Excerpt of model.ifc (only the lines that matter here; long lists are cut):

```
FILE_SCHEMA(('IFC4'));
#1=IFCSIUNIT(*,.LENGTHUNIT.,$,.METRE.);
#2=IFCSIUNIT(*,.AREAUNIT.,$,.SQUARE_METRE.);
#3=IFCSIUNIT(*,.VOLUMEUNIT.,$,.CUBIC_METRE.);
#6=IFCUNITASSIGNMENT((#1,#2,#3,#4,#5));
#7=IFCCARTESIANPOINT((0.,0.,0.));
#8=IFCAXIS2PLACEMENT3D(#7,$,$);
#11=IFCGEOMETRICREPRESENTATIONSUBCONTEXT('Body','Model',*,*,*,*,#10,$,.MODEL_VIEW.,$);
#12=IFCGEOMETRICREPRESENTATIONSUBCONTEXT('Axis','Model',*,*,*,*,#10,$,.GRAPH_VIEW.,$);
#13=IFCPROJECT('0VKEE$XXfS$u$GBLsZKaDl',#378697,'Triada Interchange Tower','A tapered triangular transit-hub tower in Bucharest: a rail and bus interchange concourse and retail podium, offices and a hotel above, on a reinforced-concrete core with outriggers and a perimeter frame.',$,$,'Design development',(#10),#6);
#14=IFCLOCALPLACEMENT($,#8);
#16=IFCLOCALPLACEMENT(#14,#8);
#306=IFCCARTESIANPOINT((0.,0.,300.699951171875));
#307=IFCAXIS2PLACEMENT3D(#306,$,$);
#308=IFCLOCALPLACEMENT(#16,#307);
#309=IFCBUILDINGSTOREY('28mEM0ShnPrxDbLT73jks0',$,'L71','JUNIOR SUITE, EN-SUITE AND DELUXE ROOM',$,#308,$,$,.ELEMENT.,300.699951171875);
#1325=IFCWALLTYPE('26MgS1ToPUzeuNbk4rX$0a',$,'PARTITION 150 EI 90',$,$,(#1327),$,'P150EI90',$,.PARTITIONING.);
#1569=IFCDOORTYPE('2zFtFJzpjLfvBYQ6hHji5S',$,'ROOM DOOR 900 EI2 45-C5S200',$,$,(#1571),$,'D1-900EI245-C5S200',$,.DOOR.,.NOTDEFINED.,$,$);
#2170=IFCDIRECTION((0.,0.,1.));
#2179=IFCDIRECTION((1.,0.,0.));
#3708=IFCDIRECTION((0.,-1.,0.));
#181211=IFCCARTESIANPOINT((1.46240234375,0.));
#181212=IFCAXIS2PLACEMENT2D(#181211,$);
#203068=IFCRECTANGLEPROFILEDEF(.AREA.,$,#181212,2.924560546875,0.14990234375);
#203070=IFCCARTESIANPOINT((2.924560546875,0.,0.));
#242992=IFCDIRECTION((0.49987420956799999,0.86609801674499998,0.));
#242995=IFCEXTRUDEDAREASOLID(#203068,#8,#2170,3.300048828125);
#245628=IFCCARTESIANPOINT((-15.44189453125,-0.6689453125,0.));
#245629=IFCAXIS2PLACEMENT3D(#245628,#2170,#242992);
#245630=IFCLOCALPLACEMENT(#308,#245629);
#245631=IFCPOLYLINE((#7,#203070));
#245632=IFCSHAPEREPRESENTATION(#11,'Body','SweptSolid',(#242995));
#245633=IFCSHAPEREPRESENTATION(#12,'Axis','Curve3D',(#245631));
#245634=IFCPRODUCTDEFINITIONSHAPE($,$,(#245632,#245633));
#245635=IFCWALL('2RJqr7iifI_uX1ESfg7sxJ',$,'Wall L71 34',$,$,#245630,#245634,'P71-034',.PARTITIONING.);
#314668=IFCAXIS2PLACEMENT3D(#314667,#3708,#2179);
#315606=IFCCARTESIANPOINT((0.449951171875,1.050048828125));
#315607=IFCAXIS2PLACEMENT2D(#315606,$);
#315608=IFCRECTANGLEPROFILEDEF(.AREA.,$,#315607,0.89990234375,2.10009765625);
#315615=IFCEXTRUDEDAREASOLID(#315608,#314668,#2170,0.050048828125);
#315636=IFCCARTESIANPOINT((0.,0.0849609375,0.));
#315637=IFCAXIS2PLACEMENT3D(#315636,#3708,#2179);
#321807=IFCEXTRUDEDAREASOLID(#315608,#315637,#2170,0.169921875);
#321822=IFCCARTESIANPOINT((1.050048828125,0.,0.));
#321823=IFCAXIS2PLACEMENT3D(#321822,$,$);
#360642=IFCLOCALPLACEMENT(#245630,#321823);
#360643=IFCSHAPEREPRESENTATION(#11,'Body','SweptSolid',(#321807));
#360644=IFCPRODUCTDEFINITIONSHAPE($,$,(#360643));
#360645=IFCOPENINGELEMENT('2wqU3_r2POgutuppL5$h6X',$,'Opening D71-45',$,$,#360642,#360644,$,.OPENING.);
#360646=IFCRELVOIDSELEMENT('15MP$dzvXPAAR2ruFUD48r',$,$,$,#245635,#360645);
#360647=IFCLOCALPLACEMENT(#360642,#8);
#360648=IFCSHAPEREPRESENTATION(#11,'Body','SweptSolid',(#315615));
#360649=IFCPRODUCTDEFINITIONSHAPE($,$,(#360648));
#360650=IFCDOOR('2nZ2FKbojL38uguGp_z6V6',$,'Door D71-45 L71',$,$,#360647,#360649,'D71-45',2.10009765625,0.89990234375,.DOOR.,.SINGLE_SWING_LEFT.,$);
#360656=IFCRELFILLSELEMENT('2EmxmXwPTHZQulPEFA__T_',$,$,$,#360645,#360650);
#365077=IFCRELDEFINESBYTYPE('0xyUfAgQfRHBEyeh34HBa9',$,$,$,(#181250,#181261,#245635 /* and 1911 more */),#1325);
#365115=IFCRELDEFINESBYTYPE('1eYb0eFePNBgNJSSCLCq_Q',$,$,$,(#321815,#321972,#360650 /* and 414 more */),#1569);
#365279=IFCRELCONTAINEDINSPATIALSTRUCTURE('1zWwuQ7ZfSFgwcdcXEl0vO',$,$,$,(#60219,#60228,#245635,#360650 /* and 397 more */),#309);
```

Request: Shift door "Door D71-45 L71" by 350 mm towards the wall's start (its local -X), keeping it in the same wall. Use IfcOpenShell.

```python
import ifcopenshell
import ifcopenshell.api.geometry
import ifcopenshell.util.placement
import ifcopenshell.util.unit

model = ifcopenshell.open("model.ifc")
unit_scale = ifcopenshell.util.unit.calculate_unit_scale(model)

door = model.by_guid("2nZ2FKbojL38uguGp_z6V6")
opening = door.FillsVoids[0].RelatingOpeningElement
wall = opening.VoidsElements[0].RelatingBuildingElement

wall_matrix = ifcopenshell.util.placement.get_local_placement(wall.ObjectPlacement)
shift = wall_matrix[:3, 0] * -0.35 / unit_scale
before = ifcopenshell.util.placement.get_local_placement(door.ObjectPlacement)[:3, 3].copy()

# The door is placed relative to its opening, so it follows when the opening moves.
matrix = ifcopenshell.util.placement.get_local_placement(opening.ObjectPlacement)
matrix[:3, 3] += shift
ifcopenshell.api.geometry.edit_object_placement(
    model, product=opening, matrix=matrix, is_si=False, should_transform_children=True
)

after = ifcopenshell.util.placement.get_local_placement(door.ObjectPlacement)[:3, 3]
print("door moved by", (after - before).round(3) + 0.0)

model.write("model_v2.ifc")
```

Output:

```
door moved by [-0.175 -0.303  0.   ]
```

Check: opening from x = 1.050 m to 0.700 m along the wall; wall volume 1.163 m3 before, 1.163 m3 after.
